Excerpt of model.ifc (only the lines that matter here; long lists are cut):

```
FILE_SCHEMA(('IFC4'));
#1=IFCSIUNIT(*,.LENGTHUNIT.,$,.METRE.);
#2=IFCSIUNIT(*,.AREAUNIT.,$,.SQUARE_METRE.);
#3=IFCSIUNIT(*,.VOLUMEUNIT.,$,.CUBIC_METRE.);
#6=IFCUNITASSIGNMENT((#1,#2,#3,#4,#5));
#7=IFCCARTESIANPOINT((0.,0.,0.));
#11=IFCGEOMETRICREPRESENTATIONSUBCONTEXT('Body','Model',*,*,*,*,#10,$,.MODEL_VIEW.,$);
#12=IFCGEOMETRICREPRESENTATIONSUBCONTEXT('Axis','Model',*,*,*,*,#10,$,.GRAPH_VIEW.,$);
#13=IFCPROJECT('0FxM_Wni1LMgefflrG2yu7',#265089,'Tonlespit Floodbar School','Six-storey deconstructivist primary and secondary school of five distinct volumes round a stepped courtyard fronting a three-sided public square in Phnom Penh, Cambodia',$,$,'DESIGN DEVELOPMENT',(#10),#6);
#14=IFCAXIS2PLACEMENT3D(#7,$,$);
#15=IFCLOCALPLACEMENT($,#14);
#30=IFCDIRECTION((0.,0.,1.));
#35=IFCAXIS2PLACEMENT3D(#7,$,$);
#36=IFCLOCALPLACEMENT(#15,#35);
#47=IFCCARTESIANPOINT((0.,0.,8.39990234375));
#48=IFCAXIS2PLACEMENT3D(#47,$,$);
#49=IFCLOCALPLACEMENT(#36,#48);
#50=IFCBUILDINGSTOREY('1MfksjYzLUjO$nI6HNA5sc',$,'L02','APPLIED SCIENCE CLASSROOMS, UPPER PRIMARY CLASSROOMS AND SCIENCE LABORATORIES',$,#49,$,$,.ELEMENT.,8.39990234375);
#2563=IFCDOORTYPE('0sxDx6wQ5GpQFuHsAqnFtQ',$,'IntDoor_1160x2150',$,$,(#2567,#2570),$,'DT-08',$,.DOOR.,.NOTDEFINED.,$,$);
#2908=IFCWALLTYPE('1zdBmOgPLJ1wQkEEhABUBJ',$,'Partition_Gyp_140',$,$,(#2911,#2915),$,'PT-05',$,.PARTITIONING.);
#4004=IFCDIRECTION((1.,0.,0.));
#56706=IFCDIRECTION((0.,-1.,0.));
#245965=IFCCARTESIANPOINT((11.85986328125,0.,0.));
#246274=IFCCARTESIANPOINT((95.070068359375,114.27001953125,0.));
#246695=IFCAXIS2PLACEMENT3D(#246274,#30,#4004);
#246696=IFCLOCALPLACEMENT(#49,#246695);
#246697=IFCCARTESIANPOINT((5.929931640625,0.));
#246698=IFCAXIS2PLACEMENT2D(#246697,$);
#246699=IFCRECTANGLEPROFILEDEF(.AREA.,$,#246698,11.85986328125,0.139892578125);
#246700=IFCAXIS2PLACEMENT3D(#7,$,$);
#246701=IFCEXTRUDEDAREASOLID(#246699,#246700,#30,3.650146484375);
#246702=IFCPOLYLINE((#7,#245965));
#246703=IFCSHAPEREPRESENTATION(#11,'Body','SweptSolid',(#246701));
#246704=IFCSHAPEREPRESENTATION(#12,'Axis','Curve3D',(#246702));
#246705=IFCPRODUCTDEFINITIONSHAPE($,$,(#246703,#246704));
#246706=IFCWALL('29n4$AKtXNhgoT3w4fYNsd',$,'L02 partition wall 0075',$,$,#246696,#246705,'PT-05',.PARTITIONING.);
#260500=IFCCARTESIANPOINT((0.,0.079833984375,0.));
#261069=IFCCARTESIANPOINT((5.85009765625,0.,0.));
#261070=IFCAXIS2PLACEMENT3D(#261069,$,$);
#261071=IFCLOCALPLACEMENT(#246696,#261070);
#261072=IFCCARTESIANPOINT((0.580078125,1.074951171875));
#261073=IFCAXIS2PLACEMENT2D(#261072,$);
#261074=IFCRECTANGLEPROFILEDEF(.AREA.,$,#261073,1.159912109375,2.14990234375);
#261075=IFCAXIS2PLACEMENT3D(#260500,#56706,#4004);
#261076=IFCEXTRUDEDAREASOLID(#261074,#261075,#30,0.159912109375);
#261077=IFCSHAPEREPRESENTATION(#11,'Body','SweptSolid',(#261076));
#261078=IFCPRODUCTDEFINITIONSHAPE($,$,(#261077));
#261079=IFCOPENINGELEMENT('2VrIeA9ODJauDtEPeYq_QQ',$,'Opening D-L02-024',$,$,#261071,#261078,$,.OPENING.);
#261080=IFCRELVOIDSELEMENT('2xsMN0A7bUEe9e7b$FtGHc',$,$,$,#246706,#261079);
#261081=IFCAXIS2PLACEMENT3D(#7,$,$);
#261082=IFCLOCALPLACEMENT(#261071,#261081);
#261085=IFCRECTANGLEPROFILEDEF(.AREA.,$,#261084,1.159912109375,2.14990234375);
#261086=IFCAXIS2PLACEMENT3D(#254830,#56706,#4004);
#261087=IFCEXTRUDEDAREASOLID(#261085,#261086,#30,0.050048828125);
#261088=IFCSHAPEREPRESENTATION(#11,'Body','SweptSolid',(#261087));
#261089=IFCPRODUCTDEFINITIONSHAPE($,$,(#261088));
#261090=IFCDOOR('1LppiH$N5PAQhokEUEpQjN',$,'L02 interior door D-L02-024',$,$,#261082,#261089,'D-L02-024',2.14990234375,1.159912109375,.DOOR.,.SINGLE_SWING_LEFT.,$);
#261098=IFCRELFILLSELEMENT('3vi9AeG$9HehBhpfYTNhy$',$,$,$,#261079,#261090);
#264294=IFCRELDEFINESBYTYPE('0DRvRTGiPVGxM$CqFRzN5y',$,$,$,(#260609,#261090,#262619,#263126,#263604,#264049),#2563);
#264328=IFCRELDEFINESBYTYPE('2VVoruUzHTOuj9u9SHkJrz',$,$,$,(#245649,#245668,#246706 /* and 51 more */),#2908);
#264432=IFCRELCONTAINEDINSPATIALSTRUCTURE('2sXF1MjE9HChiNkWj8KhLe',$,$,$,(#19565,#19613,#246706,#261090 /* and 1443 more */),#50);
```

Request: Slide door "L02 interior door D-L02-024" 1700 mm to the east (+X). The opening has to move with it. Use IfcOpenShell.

```python
import ifcopenshell
import ifcopenshell.api.geometry
import ifcopenshell.util.placement

model = ifcopenshell.open("model.ifc")

door = model.by_id(261090)
opening = door.FillsVoids[0].RelatingOpeningElement
wall = opening.VoidsElements[0].RelatingBuildingElement

wall_matrix = ifcopenshell.util.placement.get_local_placement(wall.ObjectPlacement)
shift = wall_matrix[:3, 0] * 1.7
before = ifcopenshell.util.placement.get_local_placement(door.ObjectPlacement)[:3, 3].copy()

# The door is placed relative to its opening, so it follows when the opening moves.
matrix = ifcopenshell.util.placement.get_local_placement(opening.ObjectPlacement)
matrix[:3, 3] += shift
ifcopenshell.api.geometry.edit_object_placement(
    model, product=opening, matrix=matrix, is_si=False, should_transform_children=True
)

after = ifcopenshell.util.placement.get_local_placement(door.ObjectPlacement)[:3, 3]
print("door moved by", (after - before).round(3) + 0.0)

model.write("model_updated.ifc")
```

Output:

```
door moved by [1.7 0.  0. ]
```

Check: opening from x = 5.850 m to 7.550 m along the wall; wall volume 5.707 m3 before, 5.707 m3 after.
